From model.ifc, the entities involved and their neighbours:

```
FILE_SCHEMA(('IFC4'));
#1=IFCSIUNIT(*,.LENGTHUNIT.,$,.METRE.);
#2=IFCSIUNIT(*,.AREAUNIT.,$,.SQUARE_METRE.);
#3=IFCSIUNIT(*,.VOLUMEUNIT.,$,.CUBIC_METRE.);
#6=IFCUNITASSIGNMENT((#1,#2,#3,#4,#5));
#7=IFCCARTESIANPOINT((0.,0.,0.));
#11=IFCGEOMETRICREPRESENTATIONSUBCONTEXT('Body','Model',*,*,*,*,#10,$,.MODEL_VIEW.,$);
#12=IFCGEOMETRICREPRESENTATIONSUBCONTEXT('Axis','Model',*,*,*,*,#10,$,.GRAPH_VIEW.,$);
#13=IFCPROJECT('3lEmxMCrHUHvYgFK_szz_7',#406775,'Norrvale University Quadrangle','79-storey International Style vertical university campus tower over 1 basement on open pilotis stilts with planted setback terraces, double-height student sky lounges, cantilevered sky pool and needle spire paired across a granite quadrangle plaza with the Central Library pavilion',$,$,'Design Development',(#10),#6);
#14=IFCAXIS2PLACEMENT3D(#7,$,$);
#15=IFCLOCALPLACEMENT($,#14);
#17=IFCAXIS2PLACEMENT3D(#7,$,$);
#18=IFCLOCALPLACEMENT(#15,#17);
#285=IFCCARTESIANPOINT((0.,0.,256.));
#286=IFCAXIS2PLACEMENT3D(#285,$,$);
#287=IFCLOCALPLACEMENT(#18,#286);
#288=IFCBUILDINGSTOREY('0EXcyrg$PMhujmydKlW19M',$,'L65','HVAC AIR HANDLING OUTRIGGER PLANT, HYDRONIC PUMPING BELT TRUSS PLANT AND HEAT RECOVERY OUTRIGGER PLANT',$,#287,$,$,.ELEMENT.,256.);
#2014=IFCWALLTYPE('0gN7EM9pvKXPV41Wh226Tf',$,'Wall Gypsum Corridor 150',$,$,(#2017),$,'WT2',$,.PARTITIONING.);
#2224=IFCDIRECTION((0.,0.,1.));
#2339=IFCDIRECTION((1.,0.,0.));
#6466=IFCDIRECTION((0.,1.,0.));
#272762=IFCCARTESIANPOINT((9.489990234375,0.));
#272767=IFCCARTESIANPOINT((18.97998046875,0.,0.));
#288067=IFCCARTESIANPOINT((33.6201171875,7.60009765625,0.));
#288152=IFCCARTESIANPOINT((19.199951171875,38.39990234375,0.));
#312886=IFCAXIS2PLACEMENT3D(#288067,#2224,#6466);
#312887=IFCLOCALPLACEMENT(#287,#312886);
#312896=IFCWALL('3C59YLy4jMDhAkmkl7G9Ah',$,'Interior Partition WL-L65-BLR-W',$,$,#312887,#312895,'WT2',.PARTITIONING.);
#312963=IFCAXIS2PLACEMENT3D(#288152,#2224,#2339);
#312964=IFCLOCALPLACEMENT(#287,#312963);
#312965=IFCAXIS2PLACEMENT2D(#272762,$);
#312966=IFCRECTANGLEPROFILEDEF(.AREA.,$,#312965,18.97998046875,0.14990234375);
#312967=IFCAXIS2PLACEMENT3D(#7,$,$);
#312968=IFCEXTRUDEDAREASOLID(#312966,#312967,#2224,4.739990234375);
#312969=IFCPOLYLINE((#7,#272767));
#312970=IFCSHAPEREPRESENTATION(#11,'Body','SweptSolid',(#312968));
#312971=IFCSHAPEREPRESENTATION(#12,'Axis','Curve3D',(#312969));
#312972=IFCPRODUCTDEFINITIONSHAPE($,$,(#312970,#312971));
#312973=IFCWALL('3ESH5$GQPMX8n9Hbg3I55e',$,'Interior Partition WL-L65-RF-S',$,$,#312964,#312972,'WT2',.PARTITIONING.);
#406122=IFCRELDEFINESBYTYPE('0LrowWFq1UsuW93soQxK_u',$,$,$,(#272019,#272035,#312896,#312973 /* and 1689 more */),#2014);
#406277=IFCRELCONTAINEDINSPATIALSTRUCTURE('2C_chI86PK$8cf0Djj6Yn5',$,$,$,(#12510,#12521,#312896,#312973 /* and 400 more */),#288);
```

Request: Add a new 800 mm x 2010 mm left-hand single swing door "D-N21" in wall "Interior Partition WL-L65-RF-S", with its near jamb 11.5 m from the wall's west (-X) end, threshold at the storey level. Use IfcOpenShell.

```python
import numpy as np
import ifcopenshell
import ifcopenshell.api.feature
import ifcopenshell.api.geometry
import ifcopenshell.api.root
import ifcopenshell.api.spatial
import ifcopenshell.geom
import ifcopenshell.util.element
import ifcopenshell.util.placement
import ifcopenshell.util.representation
import ifcopenshell.util.shape
import ifcopenshell.util.unit

model = ifcopenshell.open("model.ifc")
unit_scale = ifcopenshell.util.unit.calculate_unit_scale(model)
settings = ifcopenshell.geom.settings()


def volume(element):
    """Net volume in cubic metres, openings subtracted."""
    shape = ifcopenshell.geom.create_shape(settings, element)
    return ifcopenshell.util.shape.get_volume(shape.geometry)


wall = model.by_guid("3ESH5$GQPMX8n9Hbg3I55e")
storey = ifcopenshell.util.element.get_container(wall, ifc_class="IfcBuildingStorey")
context = ifcopenshell.util.representation.get_context(model, "Model", "Body", "MODEL_VIEW")
before = volume(wall)

width, height, from_end, sill = 0.8, 2.01, 11.5, 0.0  # metres

# The wall runs along its own X axis, and the end named is its -X end.
wall_shape = ifcopenshell.geom.create_shape(settings, wall)
x, y, z = ifcopenshell.util.shape.get_vertices(wall_shape.geometry).T
start = x.min() + from_end
face, thickness = float(y.min()), float(y.max() - y.min())
wall_matrix = ifcopenshell.util.placement.get_local_placement(wall.ObjectPlacement)
level = ifcopenshell.util.placement.get_local_placement(storey.ObjectPlacement)[2, 3]


def in_wall(x, y):
    """Placement at x, y metres in the wall's axes, at sill height."""
    matrix = wall_matrix.copy()
    matrix[:, 3] = wall_matrix @ np.array([x / unit_scale, y / unit_scale, 0.0, 1.0])
    matrix[2, 3] = level + sill / unit_scale
    return matrix


# Opening: a box that overshoots both wall faces by 50 mm.
opening = ifcopenshell.api.root.create_entity(model, ifc_class="IfcOpeningElement", predefined_type="OPENING")
box = ifcopenshell.api.geometry.add_wall_representation(
    model, context=context, length=width, height=height, thickness=thickness + 0.1
)
ifcopenshell.api.geometry.assign_representation(model, product=opening, representation=box)
ifcopenshell.api.geometry.edit_object_placement(model, product=opening, matrix=in_wall(start, face - 0.05), is_si=False)
ifcopenshell.api.feature.add_feature(model, feature=opening, element=wall)

door = ifcopenshell.api.root.create_entity(model, ifc_class="IfcDoor", name="D-N21", predefined_type="DOOR")
door.OverallWidth, door.OverallHeight = width / unit_scale, height / unit_scale
door.OperationType = "SINGLE_SWING_LEFT"
body = ifcopenshell.api.geometry.add_door_representation(
    model,
    context=context,
    overall_width=door.OverallWidth,
    overall_height=door.OverallHeight,
    operation_type="SINGLE_SWING_LEFT",
    lining_properties={"LiningDepth": thickness / unit_scale, "ThresholdDepth": thickness / unit_scale},
)
ifcopenshell.api.geometry.assign_representation(model, product=door, representation=body)
ifcopenshell.api.spatial.assign_container(model, products=[door], relating_structure=storey)
ifcopenshell.api.feature.add_filling(model, opening=opening, element=door)

# The lining spans the wall, so the door starts at the wall face.
ifcopenshell.api.geometry.edit_object_placement(model, product=door, matrix=in_wall(start, face), is_si=False)

after = volume(wall)

print(f"wall volume {before:.3f} -> {after:.3f} m3")

model.write("model_updated.ifc")
```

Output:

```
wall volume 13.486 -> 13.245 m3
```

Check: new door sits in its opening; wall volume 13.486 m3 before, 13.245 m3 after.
